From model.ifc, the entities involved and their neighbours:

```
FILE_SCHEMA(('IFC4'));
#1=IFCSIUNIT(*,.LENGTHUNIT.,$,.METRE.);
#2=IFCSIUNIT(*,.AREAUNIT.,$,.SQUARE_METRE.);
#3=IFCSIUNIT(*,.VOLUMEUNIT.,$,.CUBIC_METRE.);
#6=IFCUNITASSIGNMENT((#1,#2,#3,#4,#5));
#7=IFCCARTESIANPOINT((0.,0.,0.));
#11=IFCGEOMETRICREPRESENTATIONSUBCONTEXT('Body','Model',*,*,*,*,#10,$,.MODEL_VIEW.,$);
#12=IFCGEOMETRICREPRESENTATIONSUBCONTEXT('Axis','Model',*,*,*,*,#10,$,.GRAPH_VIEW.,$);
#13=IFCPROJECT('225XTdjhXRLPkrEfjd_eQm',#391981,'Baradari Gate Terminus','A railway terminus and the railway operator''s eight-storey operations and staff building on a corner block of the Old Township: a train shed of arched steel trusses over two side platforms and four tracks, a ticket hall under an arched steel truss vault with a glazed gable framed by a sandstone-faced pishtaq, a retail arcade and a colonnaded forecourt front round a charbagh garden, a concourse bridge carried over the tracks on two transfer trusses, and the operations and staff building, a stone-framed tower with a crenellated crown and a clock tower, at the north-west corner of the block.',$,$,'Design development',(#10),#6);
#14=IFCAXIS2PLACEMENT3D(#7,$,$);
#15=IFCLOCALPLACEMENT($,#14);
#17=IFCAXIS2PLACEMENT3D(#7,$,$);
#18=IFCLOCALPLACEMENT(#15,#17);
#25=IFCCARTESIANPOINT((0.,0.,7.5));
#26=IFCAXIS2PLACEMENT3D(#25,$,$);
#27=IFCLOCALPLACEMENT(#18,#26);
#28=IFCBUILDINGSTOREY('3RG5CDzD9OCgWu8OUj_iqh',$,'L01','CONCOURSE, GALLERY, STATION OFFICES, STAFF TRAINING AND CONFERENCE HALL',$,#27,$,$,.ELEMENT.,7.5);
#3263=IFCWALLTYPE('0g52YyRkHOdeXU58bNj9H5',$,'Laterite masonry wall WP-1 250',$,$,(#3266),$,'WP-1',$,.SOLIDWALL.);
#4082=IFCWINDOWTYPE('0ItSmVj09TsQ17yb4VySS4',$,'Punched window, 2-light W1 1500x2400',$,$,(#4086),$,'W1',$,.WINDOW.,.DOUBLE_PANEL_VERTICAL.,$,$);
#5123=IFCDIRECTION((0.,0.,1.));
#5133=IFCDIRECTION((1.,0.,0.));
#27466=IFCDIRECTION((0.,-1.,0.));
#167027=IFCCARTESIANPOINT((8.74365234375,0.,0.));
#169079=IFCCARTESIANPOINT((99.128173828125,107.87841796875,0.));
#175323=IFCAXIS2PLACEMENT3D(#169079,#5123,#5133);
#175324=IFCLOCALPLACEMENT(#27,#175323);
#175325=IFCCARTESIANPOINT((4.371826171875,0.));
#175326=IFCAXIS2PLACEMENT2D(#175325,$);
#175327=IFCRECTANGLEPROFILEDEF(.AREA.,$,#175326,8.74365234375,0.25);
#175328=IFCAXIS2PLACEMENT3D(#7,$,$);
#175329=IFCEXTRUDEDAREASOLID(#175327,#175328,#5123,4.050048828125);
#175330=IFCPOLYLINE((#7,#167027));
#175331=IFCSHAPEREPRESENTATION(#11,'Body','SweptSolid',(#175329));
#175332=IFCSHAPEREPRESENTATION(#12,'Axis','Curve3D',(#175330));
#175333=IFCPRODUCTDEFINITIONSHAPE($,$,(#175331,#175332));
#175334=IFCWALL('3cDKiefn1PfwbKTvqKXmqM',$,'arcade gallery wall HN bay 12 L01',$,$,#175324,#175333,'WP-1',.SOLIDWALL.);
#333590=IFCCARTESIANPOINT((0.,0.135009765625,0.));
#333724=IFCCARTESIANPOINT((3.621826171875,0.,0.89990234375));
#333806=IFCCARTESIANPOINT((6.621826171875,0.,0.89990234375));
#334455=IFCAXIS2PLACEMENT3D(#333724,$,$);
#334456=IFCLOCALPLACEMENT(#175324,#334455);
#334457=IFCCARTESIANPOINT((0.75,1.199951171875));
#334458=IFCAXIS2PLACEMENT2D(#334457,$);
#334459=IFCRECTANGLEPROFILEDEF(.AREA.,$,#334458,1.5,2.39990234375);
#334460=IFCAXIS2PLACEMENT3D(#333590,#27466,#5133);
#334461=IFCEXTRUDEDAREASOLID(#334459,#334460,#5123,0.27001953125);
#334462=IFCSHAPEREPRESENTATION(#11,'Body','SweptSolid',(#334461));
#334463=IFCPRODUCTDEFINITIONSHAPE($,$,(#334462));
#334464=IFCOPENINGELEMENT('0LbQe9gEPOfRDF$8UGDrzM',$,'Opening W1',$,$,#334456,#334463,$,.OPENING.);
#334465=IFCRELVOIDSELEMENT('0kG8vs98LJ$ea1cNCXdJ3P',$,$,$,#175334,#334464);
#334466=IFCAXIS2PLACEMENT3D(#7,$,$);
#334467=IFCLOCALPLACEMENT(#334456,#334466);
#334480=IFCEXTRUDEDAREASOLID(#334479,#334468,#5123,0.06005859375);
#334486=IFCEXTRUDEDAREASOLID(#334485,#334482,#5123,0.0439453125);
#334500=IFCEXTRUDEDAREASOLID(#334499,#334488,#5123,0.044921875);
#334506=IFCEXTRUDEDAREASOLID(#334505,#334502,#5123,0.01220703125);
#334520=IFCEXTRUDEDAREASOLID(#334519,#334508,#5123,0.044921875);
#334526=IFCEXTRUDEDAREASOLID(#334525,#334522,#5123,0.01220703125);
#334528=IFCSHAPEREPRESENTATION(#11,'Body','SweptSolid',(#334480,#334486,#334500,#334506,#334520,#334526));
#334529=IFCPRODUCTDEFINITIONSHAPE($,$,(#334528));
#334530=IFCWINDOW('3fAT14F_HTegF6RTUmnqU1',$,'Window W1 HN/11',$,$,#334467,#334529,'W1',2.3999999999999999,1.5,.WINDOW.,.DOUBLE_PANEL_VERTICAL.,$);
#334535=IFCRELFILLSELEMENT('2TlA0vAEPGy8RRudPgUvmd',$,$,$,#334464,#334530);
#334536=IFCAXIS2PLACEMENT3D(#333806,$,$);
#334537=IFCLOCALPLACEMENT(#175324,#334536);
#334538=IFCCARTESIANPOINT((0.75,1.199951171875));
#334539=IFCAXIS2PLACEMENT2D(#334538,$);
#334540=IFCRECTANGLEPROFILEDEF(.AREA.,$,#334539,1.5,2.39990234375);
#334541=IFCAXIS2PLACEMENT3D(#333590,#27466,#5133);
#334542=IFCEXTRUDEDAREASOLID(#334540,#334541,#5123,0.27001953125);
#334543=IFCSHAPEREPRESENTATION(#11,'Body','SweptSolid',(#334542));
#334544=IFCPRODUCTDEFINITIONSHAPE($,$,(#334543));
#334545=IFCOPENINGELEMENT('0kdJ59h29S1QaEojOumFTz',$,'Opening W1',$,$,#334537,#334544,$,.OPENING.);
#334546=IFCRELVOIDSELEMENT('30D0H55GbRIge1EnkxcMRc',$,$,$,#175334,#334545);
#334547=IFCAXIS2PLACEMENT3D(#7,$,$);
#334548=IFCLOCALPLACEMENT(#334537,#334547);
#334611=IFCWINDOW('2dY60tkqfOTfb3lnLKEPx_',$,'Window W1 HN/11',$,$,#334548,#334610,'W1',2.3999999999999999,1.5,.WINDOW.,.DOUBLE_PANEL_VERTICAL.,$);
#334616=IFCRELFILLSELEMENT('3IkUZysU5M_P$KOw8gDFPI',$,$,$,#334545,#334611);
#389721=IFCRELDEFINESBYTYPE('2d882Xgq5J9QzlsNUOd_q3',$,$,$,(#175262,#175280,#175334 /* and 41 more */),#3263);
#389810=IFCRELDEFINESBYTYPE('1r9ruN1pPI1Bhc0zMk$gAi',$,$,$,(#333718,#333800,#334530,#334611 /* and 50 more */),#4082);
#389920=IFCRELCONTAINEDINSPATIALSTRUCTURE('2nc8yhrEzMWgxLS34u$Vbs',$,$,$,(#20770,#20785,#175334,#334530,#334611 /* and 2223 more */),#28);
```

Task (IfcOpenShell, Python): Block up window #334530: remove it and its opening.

```python
import ifcopenshell
import ifcopenshell.api.feature
import ifcopenshell.api.root
import ifcopenshell.geom
import ifcopenshell.util.shape

model = ifcopenshell.open("model.ifc")
settings = ifcopenshell.geom.settings()


def volume(element):
    """Net volume in cubic metres, openings subtracted."""
    shape = ifcopenshell.geom.create_shape(settings, element)
    return ifcopenshell.util.shape.get_volume(shape.geometry)


window = model.by_guid("3fAT14F_HTegF6RTUmnqU1")
opening = window.FillsVoids[0].RelatingOpeningElement
wall = opening.VoidsElements[0].RelatingBuildingElement
before = volume(wall)

ifcopenshell.api.root.remove_product(model, product=window)
ifcopenshell.api.feature.remove_feature(model, feature=opening)

after = volume(wall)

print(f"wall volume {before:.3f} -> {after:.3f} m3")

model.write("model_rev.ifc")
```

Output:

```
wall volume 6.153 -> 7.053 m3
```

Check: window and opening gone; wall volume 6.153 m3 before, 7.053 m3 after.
